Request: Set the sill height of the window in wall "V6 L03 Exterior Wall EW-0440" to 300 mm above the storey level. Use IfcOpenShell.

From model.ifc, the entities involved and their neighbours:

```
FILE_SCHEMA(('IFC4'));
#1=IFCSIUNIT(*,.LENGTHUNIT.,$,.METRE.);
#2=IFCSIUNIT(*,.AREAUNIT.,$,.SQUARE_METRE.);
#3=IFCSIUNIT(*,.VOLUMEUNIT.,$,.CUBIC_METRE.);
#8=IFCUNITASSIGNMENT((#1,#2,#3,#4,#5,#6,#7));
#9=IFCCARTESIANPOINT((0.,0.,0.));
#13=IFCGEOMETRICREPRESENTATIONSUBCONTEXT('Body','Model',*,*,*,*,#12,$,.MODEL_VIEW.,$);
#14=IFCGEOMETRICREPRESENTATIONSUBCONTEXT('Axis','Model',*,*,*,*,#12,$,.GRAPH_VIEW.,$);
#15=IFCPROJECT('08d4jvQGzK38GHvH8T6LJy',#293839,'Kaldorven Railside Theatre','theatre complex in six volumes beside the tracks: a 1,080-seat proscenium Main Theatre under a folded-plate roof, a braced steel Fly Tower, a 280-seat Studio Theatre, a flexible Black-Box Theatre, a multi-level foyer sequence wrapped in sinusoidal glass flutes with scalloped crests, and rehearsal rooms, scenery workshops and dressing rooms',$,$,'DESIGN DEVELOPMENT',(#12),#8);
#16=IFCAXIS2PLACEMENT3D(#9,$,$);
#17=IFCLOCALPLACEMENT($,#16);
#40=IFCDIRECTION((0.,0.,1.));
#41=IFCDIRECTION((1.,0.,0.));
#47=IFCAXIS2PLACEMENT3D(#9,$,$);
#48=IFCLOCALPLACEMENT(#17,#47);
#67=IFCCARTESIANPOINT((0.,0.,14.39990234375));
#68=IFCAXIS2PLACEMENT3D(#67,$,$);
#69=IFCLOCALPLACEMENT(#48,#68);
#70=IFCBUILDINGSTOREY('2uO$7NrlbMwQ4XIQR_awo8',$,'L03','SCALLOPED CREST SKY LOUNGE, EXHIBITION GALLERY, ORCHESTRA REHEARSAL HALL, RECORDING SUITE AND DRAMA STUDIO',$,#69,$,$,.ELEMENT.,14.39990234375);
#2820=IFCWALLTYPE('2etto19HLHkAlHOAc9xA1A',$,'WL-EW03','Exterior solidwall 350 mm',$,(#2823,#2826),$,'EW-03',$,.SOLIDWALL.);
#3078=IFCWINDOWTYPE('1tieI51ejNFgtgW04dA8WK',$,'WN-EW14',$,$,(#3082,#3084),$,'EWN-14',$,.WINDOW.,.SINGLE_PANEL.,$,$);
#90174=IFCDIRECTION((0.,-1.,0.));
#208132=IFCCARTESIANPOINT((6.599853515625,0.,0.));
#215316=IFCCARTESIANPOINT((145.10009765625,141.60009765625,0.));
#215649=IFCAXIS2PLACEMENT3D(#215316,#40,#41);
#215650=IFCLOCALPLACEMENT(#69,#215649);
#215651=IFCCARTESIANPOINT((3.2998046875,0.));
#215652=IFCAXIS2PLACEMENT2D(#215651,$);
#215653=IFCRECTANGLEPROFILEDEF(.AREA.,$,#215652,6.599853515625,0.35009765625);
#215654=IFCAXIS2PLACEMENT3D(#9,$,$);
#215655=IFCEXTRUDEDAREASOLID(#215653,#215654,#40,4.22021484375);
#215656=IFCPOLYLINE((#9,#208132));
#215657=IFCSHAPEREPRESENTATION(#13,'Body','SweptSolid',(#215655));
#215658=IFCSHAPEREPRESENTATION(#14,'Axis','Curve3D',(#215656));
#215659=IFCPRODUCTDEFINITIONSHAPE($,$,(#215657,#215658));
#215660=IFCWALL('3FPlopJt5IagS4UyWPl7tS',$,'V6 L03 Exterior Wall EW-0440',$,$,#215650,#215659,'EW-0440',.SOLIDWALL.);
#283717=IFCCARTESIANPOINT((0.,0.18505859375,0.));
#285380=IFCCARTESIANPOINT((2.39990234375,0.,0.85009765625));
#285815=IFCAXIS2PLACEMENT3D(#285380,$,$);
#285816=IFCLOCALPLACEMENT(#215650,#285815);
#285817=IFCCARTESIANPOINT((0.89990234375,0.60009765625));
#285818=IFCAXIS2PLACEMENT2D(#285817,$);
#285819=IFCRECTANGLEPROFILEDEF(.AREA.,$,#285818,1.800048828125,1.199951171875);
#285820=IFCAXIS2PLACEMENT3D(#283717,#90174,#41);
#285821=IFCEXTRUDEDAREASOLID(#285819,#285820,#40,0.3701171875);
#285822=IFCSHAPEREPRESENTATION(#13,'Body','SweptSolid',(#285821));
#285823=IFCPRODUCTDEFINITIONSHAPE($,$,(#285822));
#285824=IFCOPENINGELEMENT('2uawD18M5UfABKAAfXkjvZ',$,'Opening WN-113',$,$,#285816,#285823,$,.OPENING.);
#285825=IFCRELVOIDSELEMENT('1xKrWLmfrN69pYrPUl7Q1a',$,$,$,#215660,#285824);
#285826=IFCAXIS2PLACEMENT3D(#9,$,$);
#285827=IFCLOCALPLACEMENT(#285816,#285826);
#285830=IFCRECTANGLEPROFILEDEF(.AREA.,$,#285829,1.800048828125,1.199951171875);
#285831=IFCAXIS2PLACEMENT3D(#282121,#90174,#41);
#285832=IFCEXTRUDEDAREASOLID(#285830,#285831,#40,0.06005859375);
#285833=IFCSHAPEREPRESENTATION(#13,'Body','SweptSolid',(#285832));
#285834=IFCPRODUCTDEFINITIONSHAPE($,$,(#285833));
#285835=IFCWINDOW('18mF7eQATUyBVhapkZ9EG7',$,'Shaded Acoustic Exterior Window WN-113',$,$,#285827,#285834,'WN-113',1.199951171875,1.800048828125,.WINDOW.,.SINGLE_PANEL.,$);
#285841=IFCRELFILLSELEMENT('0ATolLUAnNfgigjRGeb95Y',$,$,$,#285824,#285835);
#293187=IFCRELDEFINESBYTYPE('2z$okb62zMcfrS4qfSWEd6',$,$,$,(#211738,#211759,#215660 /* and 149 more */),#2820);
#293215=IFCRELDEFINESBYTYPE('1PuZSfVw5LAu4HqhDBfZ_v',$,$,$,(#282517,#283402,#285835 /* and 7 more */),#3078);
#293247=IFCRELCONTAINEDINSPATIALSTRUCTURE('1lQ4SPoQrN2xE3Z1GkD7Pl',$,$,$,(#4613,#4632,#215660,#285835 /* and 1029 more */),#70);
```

```python
import numpy as np
import ifcopenshell
import ifcopenshell.api.geometry
import ifcopenshell.geom
import ifcopenshell.util.element
import ifcopenshell.util.placement
import ifcopenshell.util.shape
import ifcopenshell.util.unit

model = ifcopenshell.open("model.ifc")
unit_scale = ifcopenshell.util.unit.calculate_unit_scale(model)

window = model.by_guid("18mF7eQATUyBVhapkZ9EG7")
opening = window.FillsVoids[0].RelatingOpeningElement
storey = ifcopenshell.util.element.get_container(window, ifc_class="IfcBuildingStorey")
level = ifcopenshell.util.placement.get_local_placement(storey.ObjectPlacement)[2, 3]

# The opening's origin need not be at the sill, so measure its lowest point.
shape = ifcopenshell.geom.create_shape(ifcopenshell.geom.settings(), opening)
bottom = ifcopenshell.util.shape.get_shape_bottom_elevation(shape, shape.geometry) / unit_scale
dz = level + 0.3 / unit_scale - bottom

shift = np.array([0.0, 0.0, dz])
# The window is placed relative to its opening, so it follows when the opening moves.
matrix = ifcopenshell.util.placement.get_local_placement(opening.ObjectPlacement)
matrix[:3, 3] += shift
ifcopenshell.api.geometry.edit_object_placement(
    model, product=opening, matrix=matrix, is_si=False, should_transform_children=True
)

print(f"moved by {dz * unit_scale:+.3f} m")

model.write("model-out.ifc")
```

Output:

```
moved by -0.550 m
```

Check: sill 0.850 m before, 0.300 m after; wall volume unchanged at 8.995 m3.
